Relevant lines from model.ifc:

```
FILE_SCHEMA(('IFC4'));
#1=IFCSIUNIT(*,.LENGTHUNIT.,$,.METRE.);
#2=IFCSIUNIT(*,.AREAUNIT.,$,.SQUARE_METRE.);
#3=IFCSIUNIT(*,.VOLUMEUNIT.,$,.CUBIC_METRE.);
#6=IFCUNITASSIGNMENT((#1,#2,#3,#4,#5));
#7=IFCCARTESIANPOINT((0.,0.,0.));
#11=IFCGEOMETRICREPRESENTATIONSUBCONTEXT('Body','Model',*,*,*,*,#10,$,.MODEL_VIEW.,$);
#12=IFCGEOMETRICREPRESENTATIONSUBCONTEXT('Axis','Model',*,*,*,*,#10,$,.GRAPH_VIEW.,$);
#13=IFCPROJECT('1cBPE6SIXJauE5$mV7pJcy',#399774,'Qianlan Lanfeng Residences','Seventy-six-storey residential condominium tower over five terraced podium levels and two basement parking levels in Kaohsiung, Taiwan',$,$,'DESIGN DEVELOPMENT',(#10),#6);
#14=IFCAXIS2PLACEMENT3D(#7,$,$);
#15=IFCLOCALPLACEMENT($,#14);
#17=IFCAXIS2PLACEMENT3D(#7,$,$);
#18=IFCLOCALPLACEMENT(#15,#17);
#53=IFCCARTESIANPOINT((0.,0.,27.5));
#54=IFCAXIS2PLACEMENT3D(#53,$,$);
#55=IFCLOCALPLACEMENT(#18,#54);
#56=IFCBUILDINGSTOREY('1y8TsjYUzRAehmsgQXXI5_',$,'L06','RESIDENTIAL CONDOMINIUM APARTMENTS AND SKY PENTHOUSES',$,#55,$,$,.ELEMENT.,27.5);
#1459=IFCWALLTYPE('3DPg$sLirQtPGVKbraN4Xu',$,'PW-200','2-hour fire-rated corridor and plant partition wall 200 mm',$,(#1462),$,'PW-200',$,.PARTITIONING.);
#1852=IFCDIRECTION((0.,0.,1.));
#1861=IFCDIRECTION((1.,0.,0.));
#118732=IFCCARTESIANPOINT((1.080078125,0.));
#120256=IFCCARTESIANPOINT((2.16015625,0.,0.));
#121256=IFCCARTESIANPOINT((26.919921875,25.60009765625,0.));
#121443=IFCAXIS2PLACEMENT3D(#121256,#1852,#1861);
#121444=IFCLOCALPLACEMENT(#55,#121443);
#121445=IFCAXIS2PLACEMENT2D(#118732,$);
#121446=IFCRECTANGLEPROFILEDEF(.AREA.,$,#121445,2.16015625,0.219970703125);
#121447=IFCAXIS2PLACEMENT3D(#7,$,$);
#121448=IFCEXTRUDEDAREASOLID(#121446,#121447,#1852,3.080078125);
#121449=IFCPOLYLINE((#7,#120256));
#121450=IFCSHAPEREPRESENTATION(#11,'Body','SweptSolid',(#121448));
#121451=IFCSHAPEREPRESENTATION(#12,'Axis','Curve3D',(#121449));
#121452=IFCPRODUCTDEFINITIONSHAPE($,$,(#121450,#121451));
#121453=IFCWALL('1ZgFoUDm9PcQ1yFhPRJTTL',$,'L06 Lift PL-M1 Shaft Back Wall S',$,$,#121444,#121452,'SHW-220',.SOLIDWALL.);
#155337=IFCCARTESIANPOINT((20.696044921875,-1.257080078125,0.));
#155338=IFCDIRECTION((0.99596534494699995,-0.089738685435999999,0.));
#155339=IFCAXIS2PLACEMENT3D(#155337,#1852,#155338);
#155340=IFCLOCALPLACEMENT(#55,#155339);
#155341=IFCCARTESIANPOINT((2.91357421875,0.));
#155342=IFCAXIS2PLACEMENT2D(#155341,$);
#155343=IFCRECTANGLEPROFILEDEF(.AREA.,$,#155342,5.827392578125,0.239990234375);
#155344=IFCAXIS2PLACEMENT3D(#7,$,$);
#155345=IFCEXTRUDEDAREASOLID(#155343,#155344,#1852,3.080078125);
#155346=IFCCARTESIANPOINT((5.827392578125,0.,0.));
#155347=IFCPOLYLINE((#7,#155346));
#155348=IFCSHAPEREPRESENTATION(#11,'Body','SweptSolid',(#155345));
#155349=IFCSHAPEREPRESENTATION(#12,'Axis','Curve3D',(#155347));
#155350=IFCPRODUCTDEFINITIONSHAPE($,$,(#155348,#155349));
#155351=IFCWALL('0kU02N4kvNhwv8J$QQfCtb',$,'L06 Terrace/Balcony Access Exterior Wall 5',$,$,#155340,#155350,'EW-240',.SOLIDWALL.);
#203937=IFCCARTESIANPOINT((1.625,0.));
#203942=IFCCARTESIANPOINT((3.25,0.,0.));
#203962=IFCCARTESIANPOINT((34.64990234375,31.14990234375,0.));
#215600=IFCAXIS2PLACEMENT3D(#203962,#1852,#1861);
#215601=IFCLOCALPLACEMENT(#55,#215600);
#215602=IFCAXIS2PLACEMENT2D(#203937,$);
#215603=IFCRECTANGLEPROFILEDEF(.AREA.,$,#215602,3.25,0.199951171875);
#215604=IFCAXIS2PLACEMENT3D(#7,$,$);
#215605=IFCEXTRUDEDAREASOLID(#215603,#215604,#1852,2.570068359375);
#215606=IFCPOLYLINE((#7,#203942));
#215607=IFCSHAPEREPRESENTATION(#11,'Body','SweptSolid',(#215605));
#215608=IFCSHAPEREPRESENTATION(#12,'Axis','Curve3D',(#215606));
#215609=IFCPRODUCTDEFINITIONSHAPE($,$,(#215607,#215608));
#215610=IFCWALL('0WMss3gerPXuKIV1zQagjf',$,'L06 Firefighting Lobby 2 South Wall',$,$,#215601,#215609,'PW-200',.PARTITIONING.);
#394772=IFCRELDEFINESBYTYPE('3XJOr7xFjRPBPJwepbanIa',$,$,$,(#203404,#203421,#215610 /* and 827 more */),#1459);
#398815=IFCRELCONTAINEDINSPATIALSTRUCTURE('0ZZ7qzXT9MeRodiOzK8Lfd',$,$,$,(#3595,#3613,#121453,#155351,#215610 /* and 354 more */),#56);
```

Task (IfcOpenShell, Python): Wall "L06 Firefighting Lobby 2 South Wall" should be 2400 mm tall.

```python
import ifcopenshell
import ifcopenshell.geom
import ifcopenshell.util.representation
import ifcopenshell.util.shape
import ifcopenshell.util.unit

model = ifcopenshell.open("model.ifc")
unit_scale = ifcopenshell.util.unit.calculate_unit_scale(model)
settings = ifcopenshell.geom.settings()


def volume(element):
    """Net volume in cubic metres, openings subtracted."""
    shape = ifcopenshell.geom.create_shape(settings, element)
    return ifcopenshell.util.shape.get_volume(shape.geometry)


wall = model.by_guid("0WMss3gerPXuKIV1zQagjf")
before = volume(wall)

body = ifcopenshell.util.representation.get_representation(wall, "Model", "Body")
solid = body.Items[0]
old_height = solid.Depth
solid.Depth = 2.4 / unit_scale
after = volume(wall)

print(f"height {old_height:g} -> {solid.Depth:g}, volume {before:.3f} -> {after:.3f} m3")

model.write("model_updated.ifc")
```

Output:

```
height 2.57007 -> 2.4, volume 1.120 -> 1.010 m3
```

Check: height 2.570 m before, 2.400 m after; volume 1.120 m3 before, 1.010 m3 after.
